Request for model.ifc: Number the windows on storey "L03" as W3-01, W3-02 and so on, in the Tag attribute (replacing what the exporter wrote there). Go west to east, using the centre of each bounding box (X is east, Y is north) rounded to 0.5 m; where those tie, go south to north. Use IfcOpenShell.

First a look at what the model holds.

```python
import ifcopenshell
import ifcopenshell.util.element
import ifcopenshell.util.placement

model = ifcopenshell.open("model.ifc")
print(model.schema)
storey = next(s for s in model.by_type("IfcBuildingStorey") if s.Name == "L03")
windows = [e for e in ifcopenshell.util.element.get_decomposition(storey) if e.is_a("IfcWindow")]
for e in sorted(windows, key=lambda e: e.id()):
    origin = ifcopenshell.util.placement.get_local_placement(e.ObjectPlacement)[:3, 3]
    print(e.id(), e.Tag, e.Name, origin.round(2) + 0.0, sep=" | ")
```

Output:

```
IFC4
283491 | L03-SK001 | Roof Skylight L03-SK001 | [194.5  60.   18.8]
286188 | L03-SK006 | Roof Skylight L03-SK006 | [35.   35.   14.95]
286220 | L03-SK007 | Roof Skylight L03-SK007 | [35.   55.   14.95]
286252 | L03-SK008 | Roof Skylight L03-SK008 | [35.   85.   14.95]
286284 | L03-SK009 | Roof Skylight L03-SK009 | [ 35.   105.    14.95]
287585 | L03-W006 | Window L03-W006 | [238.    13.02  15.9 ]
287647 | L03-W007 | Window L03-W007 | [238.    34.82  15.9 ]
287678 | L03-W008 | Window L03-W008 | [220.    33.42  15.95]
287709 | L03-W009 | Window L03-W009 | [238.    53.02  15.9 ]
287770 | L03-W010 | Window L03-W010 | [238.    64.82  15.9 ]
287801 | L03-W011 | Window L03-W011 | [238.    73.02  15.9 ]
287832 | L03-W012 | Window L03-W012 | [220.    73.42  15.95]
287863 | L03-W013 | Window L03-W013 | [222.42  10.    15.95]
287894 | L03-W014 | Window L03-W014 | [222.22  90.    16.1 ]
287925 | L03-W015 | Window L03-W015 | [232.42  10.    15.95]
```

```python
import ifcopenshell
import ifcopenshell.geom
import ifcopenshell.util.element
import ifcopenshell.util.shape

model = ifcopenshell.open("model.ifc")
settings = ifcopenshell.geom.settings()
settings.set("use-world-coords", True)


def centre(element):
    shape = ifcopenshell.geom.create_shape(settings, element)
    return ifcopenshell.util.shape.get_bbox_centroid(shape.geometry)


storey = next(s for s in model.by_type("IfcBuildingStorey") if s.Name == "L03")
windows = [e for e in ifcopenshell.util.element.get_decomposition(storey) if e.is_a("IfcWindow")]

# Insertion points can sit at a corner or the storey origin, so sort by the geometry (in metres).
centres = {e: centre(e) for e in windows}
windows.sort(key=lambda e: (round(centres[e][0] / 0.5), centres[e][1]))

for i, e in enumerate(windows, start=1):
    number = f"W3-{i:02d}"
    e.Tag = number
    print(e.id(), number)

model.write("model_v2.ifc")
```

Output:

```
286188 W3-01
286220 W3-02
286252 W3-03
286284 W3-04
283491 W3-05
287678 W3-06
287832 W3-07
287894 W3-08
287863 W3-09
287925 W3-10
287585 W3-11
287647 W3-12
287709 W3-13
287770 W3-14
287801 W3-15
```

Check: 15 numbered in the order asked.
